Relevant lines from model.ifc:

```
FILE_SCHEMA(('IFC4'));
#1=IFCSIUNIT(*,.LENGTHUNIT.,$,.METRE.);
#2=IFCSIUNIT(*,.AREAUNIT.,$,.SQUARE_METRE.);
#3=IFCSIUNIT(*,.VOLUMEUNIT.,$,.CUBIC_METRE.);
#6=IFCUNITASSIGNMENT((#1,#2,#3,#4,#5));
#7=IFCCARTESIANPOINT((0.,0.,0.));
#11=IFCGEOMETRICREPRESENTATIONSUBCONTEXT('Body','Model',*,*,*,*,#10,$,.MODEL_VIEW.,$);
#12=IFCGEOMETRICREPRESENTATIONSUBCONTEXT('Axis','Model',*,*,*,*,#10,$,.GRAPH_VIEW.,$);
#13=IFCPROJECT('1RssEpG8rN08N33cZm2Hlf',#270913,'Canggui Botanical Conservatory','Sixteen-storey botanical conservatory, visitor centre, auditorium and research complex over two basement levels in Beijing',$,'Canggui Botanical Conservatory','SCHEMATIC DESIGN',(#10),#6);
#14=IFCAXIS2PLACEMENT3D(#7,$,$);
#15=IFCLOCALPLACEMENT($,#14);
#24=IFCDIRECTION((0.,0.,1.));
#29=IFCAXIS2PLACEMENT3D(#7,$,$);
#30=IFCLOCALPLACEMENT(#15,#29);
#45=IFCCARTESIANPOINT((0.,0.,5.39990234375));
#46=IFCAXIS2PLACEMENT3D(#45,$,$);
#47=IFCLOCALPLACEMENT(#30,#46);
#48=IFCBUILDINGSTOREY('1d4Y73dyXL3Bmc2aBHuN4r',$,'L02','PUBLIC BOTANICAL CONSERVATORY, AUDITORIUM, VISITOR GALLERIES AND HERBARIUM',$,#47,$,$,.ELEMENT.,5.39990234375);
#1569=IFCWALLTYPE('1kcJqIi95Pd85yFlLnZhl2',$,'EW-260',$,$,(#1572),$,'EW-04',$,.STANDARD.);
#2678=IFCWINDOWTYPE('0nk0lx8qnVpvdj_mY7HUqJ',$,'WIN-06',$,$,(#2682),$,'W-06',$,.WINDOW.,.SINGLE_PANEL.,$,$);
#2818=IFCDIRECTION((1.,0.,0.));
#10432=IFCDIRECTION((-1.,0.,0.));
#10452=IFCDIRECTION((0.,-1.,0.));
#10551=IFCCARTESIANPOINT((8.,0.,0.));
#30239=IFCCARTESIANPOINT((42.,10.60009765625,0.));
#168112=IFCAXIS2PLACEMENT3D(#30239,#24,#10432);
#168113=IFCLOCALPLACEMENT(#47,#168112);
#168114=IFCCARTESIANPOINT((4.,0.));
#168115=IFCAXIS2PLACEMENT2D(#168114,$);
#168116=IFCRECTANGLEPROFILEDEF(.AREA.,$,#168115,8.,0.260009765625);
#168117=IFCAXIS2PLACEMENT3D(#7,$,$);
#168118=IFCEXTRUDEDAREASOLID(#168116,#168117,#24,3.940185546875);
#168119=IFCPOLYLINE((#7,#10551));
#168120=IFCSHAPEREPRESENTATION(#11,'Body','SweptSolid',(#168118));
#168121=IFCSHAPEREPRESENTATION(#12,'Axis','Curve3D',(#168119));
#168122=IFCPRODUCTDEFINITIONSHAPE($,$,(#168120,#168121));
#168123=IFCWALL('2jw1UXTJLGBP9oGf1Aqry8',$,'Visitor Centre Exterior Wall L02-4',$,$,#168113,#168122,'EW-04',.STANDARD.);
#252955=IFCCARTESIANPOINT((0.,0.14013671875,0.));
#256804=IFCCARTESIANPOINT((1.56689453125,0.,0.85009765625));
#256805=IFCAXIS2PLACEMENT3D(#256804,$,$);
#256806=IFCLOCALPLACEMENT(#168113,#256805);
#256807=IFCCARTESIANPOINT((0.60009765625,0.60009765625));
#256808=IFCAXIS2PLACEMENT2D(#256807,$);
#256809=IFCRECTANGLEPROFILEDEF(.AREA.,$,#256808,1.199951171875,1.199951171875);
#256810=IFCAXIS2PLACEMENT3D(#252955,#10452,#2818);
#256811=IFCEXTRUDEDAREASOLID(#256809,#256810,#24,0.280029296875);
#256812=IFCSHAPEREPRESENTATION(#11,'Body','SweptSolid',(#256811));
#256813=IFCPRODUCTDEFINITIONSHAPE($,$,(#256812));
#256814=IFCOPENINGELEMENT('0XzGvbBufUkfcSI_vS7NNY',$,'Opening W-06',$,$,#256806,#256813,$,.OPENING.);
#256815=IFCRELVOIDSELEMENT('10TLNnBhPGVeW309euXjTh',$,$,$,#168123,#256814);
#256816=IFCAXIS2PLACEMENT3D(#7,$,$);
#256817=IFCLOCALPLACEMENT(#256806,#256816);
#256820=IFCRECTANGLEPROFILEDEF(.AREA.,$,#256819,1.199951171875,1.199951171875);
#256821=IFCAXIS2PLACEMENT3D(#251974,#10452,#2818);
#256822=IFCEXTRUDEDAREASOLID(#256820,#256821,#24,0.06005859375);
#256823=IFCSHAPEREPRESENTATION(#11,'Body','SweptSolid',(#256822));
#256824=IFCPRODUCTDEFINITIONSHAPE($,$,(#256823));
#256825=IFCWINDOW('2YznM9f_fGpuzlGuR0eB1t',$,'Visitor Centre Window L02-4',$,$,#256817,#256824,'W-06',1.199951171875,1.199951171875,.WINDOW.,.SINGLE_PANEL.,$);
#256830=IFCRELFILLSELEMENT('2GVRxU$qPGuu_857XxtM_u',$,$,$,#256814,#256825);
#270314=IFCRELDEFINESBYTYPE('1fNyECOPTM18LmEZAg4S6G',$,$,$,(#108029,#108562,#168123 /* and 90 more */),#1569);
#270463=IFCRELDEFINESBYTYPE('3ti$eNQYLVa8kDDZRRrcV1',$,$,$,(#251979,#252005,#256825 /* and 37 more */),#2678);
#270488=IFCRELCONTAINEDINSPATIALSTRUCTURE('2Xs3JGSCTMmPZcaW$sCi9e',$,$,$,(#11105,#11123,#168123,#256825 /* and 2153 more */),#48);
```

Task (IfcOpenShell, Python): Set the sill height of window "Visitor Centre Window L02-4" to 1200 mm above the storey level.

```python
import numpy as np
import ifcopenshell
import ifcopenshell.api.geometry
import ifcopenshell.geom
import ifcopenshell.util.element
import ifcopenshell.util.placement
import ifcopenshell.util.shape
import ifcopenshell.util.unit

model = ifcopenshell.open("model.ifc")
unit_scale = ifcopenshell.util.unit.calculate_unit_scale(model)

window = model.by_id(256825)
opening = window.FillsVoids[0].RelatingOpeningElement
storey = ifcopenshell.util.element.get_container(window, ifc_class="IfcBuildingStorey")
level = ifcopenshell.util.placement.get_local_placement(storey.ObjectPlacement)[2, 3]

# The opening's origin need not be at the sill, so measure its lowest point.
shape = ifcopenshell.geom.create_shape(ifcopenshell.geom.settings(), opening)
bottom = ifcopenshell.util.shape.get_shape_bottom_elevation(shape, shape.geometry) / unit_scale
dz = level + 1.2 - bottom

shift = np.array([0.0, 0.0, dz])
# The window is placed relative to its opening, so it follows when the opening moves.
matrix = ifcopenshell.util.placement.get_local_placement(opening.ObjectPlacement)
matrix[:3, 3] += shift
ifcopenshell.api.geometry.edit_object_placement(
    model, product=opening, matrix=matrix, is_si=False, should_transform_children=True
)

print(f"moved by {dz * unit_scale:+.3f} m")

model.write("model_rev.ifc")
```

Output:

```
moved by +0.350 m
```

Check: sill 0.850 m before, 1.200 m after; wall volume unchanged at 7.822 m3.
